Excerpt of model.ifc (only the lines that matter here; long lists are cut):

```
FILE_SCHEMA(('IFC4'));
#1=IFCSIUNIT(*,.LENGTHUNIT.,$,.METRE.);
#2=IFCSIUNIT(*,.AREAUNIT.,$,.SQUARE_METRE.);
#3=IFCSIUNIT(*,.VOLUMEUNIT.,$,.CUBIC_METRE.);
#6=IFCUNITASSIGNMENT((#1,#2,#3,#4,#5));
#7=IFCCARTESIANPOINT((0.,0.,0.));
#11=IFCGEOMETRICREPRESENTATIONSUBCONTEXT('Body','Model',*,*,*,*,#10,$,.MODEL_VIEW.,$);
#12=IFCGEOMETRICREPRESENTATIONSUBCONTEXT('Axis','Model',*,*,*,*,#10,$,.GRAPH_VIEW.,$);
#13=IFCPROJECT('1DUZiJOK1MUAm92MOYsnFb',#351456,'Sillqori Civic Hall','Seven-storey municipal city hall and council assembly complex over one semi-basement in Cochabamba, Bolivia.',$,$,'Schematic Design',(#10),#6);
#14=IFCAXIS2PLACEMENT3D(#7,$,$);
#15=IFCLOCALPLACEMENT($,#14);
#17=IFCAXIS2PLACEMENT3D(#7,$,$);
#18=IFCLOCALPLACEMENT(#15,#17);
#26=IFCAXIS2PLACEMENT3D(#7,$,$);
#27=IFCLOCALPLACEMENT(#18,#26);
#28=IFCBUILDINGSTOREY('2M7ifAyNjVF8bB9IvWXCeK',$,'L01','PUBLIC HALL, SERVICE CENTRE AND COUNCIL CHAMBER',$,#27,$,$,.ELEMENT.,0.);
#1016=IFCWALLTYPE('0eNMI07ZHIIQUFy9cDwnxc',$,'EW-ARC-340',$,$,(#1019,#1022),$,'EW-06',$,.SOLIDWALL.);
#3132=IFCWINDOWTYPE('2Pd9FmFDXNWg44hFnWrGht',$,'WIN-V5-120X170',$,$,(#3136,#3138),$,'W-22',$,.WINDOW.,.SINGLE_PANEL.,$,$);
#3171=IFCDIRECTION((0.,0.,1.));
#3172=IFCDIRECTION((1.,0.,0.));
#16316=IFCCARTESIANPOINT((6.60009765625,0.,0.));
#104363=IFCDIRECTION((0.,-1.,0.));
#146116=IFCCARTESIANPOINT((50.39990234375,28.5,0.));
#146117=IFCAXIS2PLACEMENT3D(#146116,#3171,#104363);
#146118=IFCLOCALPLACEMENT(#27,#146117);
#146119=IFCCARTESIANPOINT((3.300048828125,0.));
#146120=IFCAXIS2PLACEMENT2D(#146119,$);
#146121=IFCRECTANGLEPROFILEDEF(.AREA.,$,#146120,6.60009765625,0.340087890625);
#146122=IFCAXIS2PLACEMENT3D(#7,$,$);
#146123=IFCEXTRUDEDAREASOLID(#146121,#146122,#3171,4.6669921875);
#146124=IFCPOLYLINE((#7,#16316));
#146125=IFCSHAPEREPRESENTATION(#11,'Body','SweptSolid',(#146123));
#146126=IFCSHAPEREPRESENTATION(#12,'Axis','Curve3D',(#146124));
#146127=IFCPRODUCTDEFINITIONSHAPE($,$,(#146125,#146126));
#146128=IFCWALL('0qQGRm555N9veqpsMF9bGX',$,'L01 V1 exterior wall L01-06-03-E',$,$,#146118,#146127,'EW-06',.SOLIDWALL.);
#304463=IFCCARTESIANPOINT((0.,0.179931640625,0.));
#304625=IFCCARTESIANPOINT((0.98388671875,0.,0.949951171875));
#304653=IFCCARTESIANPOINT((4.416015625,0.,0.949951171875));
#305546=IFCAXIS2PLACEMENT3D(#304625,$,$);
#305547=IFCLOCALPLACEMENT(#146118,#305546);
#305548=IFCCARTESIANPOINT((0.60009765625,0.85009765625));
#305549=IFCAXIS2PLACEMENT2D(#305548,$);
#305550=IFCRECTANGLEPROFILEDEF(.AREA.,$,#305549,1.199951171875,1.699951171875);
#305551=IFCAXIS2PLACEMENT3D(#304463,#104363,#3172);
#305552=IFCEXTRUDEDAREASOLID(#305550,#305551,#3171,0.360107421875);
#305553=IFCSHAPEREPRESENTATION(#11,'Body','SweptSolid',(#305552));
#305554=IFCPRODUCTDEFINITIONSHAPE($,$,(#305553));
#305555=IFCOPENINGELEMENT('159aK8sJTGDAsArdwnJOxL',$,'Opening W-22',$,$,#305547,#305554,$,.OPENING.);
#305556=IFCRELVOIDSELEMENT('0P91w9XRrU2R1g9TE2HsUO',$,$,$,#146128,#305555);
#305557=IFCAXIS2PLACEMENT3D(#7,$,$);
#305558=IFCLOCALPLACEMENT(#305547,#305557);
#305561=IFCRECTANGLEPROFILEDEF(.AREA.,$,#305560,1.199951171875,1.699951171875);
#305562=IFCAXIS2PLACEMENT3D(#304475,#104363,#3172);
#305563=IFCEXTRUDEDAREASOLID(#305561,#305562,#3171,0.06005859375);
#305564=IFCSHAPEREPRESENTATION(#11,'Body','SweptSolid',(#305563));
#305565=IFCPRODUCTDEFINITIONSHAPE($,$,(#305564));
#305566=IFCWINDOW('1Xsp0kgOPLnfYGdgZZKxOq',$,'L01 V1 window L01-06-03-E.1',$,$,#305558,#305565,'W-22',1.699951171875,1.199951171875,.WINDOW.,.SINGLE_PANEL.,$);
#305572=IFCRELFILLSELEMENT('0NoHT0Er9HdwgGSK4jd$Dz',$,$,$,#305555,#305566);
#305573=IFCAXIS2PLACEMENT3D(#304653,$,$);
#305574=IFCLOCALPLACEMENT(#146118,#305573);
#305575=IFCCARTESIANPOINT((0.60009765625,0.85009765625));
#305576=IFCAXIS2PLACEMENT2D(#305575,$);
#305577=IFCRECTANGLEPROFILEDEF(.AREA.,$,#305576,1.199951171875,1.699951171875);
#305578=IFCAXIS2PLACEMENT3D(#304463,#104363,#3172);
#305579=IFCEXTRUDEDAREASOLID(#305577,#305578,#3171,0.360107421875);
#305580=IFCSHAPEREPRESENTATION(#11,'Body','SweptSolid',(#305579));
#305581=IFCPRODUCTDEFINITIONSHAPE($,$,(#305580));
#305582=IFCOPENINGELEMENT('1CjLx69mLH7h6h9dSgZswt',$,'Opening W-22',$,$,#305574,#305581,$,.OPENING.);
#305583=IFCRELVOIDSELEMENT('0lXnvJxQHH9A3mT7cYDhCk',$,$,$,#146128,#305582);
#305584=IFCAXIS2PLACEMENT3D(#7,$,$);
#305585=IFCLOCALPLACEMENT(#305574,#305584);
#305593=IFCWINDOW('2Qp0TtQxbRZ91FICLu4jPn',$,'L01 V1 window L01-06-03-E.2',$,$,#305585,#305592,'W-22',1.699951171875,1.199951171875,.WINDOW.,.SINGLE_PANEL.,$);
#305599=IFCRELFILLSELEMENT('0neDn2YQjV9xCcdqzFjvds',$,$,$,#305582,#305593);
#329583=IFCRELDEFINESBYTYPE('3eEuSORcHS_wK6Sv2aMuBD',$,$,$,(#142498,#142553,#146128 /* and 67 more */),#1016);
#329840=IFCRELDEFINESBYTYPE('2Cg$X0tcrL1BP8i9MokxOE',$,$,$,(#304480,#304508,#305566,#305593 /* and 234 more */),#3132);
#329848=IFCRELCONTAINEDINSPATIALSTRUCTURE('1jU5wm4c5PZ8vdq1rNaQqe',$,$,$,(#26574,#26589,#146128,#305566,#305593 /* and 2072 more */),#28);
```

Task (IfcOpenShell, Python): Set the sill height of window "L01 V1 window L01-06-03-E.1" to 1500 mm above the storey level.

```python
import numpy as np
import ifcopenshell
import ifcopenshell.api.geometry
import ifcopenshell.geom
import ifcopenshell.util.element
import ifcopenshell.util.placement
import ifcopenshell.util.shape
import ifcopenshell.util.unit

model = ifcopenshell.open("model.ifc")
unit_scale = ifcopenshell.util.unit.calculate_unit_scale(model)

window = model.by_guid("1Xsp0kgOPLnfYGdgZZKxOq")
opening = window.FillsVoids[0].RelatingOpeningElement
storey = ifcopenshell.util.element.get_container(window, ifc_class="IfcBuildingStorey")
level = ifcopenshell.util.placement.get_local_placement(storey.ObjectPlacement)[2, 3]

# The opening's origin need not be at the sill, so measure its lowest point.
shape = ifcopenshell.geom.create_shape(ifcopenshell.geom.settings(), opening)
bottom = ifcopenshell.util.shape.get_shape_bottom_elevation(shape, shape.geometry) / unit_scale
dz = level + 1.5 / unit_scale - bottom

shift = np.array([0.0, 0.0, dz])
# The window is placed relative to its opening, so it follows when the opening moves.
matrix = ifcopenshell.util.placement.get_local_placement(opening.ObjectPlacement)
matrix[:3, 3] += shift
ifcopenshell.api.geometry.edit_object_placement(
    model, product=opening, matrix=matrix, is_si=False, should_transform_children=True
)

print(f"moved by {dz * unit_scale:+.3f} m")

model.write("model_edited.ifc")
```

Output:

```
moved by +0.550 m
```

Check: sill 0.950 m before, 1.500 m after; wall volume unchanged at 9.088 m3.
